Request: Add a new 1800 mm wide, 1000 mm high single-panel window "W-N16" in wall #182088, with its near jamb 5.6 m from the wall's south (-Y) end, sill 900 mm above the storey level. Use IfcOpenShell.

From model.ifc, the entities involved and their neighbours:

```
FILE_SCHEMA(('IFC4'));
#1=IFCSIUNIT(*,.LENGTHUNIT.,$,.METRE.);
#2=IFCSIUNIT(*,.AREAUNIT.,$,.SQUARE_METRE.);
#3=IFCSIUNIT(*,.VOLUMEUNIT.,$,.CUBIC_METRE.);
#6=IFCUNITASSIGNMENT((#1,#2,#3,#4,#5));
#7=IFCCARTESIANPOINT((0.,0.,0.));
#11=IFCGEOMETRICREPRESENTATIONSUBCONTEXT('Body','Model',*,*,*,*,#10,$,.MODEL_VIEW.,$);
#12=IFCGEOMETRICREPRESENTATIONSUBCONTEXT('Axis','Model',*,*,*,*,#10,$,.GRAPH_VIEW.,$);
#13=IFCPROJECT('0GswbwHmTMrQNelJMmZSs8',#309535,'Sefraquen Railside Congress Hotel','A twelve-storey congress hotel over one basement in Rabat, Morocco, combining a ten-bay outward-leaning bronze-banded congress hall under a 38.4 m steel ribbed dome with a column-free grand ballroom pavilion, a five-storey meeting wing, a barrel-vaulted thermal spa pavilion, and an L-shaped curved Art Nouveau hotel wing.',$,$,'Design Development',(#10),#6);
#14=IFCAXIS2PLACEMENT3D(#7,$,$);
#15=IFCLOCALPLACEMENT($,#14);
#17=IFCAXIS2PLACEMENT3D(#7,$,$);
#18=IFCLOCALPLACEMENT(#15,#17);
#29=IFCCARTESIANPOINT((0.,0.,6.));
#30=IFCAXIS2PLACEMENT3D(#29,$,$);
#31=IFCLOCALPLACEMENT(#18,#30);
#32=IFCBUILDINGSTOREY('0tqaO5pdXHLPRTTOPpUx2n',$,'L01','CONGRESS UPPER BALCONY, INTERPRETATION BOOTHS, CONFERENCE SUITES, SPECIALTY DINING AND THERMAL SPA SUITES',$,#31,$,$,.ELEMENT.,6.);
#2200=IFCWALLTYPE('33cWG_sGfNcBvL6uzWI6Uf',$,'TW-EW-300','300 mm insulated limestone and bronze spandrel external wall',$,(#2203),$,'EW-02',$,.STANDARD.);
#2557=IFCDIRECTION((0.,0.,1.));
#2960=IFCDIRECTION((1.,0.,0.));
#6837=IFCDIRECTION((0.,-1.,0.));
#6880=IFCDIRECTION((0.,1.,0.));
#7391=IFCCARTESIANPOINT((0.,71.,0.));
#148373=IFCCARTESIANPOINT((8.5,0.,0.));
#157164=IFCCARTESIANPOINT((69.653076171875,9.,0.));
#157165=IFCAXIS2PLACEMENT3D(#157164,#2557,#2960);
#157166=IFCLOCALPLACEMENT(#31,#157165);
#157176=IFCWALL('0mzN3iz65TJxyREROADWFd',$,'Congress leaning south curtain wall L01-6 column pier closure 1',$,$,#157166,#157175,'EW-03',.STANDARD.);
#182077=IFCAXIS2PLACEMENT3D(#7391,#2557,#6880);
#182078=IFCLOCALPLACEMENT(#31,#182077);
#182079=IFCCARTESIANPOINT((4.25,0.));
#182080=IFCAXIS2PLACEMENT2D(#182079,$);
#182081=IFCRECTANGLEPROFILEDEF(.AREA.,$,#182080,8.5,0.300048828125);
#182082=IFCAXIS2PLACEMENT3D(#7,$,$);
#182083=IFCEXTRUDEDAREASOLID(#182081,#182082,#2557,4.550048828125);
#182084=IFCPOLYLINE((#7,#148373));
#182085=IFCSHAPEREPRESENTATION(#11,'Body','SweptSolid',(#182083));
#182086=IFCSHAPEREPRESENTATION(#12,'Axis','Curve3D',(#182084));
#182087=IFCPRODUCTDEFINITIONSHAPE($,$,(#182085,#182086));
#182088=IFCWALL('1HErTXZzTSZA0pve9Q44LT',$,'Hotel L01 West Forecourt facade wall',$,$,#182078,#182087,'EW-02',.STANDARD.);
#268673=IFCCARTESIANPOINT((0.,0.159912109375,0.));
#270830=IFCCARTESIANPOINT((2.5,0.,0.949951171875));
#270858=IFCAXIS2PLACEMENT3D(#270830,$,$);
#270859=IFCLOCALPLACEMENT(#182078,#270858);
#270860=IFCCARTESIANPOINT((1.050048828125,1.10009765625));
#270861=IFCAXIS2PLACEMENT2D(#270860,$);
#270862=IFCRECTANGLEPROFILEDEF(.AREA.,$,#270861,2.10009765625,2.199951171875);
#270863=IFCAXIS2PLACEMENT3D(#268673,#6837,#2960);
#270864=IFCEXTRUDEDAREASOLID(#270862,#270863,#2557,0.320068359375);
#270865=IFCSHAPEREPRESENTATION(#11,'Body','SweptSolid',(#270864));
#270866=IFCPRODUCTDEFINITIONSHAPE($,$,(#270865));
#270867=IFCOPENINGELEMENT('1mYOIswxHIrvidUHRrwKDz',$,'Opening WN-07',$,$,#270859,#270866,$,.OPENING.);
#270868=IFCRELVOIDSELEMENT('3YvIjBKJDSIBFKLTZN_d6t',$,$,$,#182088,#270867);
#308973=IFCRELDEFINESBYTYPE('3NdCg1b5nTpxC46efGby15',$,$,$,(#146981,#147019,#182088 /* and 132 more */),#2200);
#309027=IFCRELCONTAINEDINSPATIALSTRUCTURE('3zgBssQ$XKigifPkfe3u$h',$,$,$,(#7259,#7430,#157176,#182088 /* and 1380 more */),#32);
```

```python
import numpy as np
import ifcopenshell
import ifcopenshell.api.feature
import ifcopenshell.api.geometry
import ifcopenshell.api.root
import ifcopenshell.api.spatial
import ifcopenshell.geom
import ifcopenshell.util.element
import ifcopenshell.util.placement
import ifcopenshell.util.representation
import ifcopenshell.util.shape
import ifcopenshell.util.unit

model = ifcopenshell.open("model.ifc")
unit_scale = ifcopenshell.util.unit.calculate_unit_scale(model)
settings = ifcopenshell.geom.settings()


def volume(element):
    """Net volume in cubic metres, openings subtracted."""
    shape = ifcopenshell.geom.create_shape(settings, element)
    return ifcopenshell.util.shape.get_volume(shape.geometry)


wall = model.by_guid("1HErTXZzTSZA0pve9Q44LT")
storey = ifcopenshell.util.element.get_container(wall, ifc_class="IfcBuildingStorey")
context = ifcopenshell.util.representation.get_context(model, "Model", "Body", "MODEL_VIEW")
before = volume(wall)

width, height, from_end, sill = 1.8, 1, 5.6, 0.9  # metres

# The wall runs along its own X axis, and the end named is its -X end.
wall_shape = ifcopenshell.geom.create_shape(settings, wall)
x, y, z = ifcopenshell.util.shape.get_vertices(wall_shape.geometry).T
start = x.min() + from_end
face, thickness = float(y.min()), float(y.max() - y.min())
wall_matrix = ifcopenshell.util.placement.get_local_placement(wall.ObjectPlacement)
level = ifcopenshell.util.placement.get_local_placement(storey.ObjectPlacement)[2, 3]


def in_wall(x, y):
    """Placement at x, y metres in the wall's axes, at sill height."""
    matrix = wall_matrix.copy()
    matrix[:, 3] = wall_matrix @ np.array([x / unit_scale, y / unit_scale, 0.0, 1.0])
    matrix[2, 3] = level + sill / unit_scale
    return matrix


# Opening: a box that overshoots both wall faces by 50 mm.
opening = ifcopenshell.api.root.create_entity(model, ifc_class="IfcOpeningElement", predefined_type="OPENING")
box = ifcopenshell.api.geometry.add_wall_representation(
    model, context=context, length=width, height=height, thickness=thickness + 0.1
)
ifcopenshell.api.geometry.assign_representation(model, product=opening, representation=box)
ifcopenshell.api.geometry.edit_object_placement(model, product=opening, matrix=in_wall(start, face - 0.05), is_si=False)
ifcopenshell.api.feature.add_feature(model, feature=opening, element=wall)

window = ifcopenshell.api.root.create_entity(model, ifc_class="IfcWindow", name="W-N16", predefined_type="WINDOW")
window.OverallWidth, window.OverallHeight = width / unit_scale, height / unit_scale
window.PartitioningType = "SINGLE_PANEL"
body = ifcopenshell.api.geometry.add_window_representation(
    model,
    context=context,
    overall_width=window.OverallWidth,
    overall_height=window.OverallHeight,
    partition_type="SINGLE_PANEL",
)
ifcopenshell.api.geometry.assign_representation(model, product=window, representation=body)
ifcopenshell.api.spatial.assign_container(model, products=[window], relating_structure=storey)
ifcopenshell.api.feature.add_filling(model, opening=opening, element=window)

# Centre the window in the wall's thickness.
ifcopenshell.api.geometry.edit_object_placement(model, product=window, matrix=in_wall(start, face), is_si=False)
window_shape = ifcopenshell.geom.create_shape(settings, window)
depth = ifcopenshell.util.shape.get_vertices(window_shape.geometry)[:, 1]
offset = face + thickness / 2 - (depth.min() + depth.max()) / 2
ifcopenshell.api.geometry.edit_object_placement(model, product=window, matrix=in_wall(start, offset), is_si=False)

after = volume(wall)

print(f"wall volume {before:.3f} -> {after:.3f} m3")

model.write("model_edited.ifc")
```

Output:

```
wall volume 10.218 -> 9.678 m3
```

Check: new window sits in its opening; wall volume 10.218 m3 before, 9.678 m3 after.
